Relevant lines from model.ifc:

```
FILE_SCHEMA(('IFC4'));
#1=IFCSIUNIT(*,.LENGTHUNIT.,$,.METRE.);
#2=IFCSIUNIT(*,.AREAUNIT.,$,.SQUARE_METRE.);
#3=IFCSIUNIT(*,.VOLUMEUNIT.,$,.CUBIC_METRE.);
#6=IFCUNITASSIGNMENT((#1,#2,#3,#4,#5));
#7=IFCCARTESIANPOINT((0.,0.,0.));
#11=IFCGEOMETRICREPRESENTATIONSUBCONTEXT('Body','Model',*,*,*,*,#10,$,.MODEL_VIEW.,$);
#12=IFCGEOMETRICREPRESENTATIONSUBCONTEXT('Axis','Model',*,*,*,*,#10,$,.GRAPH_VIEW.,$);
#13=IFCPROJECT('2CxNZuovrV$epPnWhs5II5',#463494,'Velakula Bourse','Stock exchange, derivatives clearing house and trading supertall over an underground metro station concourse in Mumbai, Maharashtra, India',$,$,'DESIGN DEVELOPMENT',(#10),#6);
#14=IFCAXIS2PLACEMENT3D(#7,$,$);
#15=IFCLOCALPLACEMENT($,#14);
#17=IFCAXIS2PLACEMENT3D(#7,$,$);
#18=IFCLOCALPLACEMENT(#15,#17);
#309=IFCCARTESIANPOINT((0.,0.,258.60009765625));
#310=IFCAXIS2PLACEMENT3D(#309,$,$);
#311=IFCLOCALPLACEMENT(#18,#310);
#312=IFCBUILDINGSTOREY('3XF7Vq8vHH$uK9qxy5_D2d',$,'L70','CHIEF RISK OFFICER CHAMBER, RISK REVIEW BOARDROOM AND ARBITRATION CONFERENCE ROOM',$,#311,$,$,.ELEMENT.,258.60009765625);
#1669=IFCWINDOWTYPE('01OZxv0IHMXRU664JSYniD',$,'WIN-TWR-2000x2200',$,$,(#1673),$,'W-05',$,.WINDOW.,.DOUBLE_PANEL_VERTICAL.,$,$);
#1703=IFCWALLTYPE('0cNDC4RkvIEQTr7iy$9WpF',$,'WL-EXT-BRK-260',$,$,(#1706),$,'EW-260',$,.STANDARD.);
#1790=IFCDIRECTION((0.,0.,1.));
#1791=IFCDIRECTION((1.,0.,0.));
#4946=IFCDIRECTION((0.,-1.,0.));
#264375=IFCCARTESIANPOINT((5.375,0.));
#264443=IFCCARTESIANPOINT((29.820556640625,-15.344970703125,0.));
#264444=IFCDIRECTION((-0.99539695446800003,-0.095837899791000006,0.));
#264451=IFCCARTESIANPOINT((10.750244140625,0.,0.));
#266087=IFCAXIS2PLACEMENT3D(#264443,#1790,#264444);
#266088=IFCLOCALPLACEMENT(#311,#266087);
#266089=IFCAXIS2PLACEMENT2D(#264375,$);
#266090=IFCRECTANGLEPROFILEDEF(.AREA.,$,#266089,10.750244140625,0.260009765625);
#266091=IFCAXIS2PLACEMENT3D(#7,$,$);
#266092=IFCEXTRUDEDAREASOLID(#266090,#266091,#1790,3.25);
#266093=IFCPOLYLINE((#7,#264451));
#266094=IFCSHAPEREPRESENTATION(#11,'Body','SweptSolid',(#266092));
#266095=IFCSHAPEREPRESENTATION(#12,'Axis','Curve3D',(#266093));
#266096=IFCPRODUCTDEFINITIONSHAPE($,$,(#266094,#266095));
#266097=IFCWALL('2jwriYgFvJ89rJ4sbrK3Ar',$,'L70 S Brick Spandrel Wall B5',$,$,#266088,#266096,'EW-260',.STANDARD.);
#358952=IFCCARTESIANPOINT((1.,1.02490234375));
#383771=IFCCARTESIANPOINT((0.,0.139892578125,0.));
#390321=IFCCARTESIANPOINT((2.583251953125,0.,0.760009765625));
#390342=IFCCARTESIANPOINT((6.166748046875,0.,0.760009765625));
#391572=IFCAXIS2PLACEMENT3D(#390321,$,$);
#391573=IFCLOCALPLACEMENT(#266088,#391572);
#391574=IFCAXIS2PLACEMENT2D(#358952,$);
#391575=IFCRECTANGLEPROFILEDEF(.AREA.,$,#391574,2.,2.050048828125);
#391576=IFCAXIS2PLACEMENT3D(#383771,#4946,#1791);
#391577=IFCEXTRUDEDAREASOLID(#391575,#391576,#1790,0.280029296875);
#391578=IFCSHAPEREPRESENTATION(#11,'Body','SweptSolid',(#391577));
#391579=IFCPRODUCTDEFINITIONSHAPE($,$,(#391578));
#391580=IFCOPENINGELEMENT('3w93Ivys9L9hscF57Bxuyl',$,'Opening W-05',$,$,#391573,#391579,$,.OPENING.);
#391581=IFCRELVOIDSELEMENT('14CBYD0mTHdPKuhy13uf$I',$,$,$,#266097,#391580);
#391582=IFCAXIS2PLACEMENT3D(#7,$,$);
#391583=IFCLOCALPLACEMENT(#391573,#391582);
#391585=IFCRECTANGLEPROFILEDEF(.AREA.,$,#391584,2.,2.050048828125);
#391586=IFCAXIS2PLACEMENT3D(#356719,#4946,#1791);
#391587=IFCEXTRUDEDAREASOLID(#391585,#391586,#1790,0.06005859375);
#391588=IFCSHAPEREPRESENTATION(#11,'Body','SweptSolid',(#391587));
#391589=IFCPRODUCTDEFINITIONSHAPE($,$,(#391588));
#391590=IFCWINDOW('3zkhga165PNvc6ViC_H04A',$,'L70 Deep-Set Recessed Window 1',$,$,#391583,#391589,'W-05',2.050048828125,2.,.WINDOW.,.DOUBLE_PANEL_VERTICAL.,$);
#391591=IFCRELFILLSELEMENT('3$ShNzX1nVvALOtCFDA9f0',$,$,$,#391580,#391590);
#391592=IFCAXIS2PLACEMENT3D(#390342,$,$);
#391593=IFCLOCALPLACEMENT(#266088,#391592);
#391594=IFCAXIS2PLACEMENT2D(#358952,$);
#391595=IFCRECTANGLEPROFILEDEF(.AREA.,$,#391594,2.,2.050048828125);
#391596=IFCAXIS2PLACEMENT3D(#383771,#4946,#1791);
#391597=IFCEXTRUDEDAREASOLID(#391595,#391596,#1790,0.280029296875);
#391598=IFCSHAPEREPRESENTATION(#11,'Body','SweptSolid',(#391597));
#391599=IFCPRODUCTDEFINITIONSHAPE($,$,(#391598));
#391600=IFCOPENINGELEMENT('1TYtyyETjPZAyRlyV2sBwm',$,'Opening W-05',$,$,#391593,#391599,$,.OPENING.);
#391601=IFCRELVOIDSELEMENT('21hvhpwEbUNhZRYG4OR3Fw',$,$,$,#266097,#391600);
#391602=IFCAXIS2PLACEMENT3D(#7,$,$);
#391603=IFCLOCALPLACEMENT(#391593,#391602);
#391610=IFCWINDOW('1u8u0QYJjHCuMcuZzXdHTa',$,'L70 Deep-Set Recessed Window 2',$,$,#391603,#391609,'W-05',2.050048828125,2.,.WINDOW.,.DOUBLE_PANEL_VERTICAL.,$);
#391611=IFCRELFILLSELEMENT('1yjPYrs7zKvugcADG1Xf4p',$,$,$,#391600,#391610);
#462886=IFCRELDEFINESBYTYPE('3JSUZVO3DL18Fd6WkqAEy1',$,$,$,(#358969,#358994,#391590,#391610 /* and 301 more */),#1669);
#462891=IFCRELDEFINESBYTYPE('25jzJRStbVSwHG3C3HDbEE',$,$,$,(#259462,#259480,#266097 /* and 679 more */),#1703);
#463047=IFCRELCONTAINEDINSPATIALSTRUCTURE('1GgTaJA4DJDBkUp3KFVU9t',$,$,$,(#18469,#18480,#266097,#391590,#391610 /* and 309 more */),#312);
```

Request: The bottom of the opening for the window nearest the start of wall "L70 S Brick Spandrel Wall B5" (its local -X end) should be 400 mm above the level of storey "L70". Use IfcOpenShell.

```python
import numpy as np
import ifcopenshell
import ifcopenshell.api.geometry
import ifcopenshell.geom
import ifcopenshell.util.element
import ifcopenshell.util.placement
import ifcopenshell.util.shape
import ifcopenshell.util.unit

model = ifcopenshell.open("model.ifc")
unit_scale = ifcopenshell.util.unit.calculate_unit_scale(model)

window = model.by_id(391590)
opening = window.FillsVoids[0].RelatingOpeningElement
storey = ifcopenshell.util.element.get_container(window, ifc_class="IfcBuildingStorey")
level = ifcopenshell.util.placement.get_local_placement(storey.ObjectPlacement)[2, 3]

# The opening's origin need not be at the sill, so measure its lowest point.
shape = ifcopenshell.geom.create_shape(ifcopenshell.geom.settings(), opening)
bottom = ifcopenshell.util.shape.get_shape_bottom_elevation(shape, shape.geometry) / unit_scale
dz = level + 0.4 - bottom

shift = np.array([0.0, 0.0, dz])
# The window is placed relative to its opening, so it follows when the opening moves.
matrix = ifcopenshell.util.placement.get_local_placement(opening.ObjectPlacement)
matrix[:3, 3] += shift
ifcopenshell.api.geometry.edit_object_placement(
    model, product=opening, matrix=matrix, is_si=False, should_transform_children=True
)

print(f"moved by {dz * unit_scale:+.3f} m")

model.write("model_rev.ifc")
```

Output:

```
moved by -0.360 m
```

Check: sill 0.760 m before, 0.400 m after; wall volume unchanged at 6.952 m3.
